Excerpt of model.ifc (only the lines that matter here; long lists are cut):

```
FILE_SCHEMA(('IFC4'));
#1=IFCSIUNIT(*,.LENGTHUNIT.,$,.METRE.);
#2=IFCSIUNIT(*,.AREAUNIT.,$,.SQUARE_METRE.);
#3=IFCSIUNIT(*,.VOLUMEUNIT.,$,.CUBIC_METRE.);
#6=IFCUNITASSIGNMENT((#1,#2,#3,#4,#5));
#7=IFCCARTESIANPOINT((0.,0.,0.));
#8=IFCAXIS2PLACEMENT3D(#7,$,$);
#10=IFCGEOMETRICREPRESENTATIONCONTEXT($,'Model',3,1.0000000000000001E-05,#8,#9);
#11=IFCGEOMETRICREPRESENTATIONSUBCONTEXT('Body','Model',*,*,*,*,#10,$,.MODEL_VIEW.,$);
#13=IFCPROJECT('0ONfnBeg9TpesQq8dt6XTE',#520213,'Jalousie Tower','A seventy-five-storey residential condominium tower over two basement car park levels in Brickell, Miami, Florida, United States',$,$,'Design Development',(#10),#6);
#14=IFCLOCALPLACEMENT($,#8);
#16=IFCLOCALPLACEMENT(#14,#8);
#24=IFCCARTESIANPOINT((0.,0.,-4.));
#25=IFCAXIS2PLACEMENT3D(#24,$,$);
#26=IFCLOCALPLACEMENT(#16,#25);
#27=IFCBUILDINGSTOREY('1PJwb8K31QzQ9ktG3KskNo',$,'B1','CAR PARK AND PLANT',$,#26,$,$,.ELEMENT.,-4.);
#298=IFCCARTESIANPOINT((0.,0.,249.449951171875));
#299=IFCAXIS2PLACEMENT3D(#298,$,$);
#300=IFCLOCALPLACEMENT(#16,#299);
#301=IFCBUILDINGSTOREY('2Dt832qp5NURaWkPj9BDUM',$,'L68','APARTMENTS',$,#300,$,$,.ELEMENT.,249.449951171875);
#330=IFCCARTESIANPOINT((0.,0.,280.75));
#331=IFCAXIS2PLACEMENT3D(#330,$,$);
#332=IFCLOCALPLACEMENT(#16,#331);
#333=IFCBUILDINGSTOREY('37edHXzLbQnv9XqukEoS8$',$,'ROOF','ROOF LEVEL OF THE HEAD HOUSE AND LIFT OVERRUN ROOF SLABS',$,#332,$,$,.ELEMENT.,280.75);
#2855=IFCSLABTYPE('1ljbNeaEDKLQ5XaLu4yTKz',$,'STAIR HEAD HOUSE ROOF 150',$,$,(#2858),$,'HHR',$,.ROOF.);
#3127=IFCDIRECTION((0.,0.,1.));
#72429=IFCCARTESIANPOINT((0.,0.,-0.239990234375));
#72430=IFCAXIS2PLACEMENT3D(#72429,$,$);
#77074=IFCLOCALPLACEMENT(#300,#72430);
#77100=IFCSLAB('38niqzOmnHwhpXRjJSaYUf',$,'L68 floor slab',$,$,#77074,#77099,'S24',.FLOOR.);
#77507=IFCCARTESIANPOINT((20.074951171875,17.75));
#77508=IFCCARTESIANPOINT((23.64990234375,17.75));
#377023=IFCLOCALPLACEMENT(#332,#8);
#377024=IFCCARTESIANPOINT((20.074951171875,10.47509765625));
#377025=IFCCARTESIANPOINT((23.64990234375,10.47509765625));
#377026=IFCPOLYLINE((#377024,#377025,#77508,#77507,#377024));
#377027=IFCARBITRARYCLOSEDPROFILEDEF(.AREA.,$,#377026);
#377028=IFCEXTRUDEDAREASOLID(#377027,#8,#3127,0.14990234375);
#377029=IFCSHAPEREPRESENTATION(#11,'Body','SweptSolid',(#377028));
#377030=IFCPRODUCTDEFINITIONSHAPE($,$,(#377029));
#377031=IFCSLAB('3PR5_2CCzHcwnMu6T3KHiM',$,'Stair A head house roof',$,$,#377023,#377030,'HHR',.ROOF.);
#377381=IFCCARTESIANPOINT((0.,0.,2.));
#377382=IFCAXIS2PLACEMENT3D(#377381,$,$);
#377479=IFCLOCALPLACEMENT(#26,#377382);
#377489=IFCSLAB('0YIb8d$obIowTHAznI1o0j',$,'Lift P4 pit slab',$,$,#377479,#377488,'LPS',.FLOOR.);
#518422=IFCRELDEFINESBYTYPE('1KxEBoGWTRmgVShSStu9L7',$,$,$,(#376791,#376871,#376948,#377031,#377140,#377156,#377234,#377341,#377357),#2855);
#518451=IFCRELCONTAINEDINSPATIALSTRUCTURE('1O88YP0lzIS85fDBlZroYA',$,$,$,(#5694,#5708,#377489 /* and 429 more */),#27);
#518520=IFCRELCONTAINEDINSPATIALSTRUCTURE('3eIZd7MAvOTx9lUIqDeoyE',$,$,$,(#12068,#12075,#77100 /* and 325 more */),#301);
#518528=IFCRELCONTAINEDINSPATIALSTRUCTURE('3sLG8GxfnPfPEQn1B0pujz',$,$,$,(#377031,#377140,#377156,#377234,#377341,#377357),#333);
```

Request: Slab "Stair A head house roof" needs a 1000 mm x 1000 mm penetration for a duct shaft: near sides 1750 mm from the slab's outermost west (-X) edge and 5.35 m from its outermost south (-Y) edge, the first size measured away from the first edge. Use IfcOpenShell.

```python
import numpy as np
import ifcopenshell
import ifcopenshell.api.feature
import ifcopenshell.api.geometry
import ifcopenshell.api.root
import ifcopenshell.geom
import ifcopenshell.util.placement
import ifcopenshell.util.representation
import ifcopenshell.util.shape
import ifcopenshell.util.unit

model = ifcopenshell.open("model.ifc")
unit_scale = ifcopenshell.util.unit.calculate_unit_scale(model)
settings = ifcopenshell.geom.settings()


def volume(element):
    """Net volume in cubic metres, openings subtracted."""
    shape = ifcopenshell.geom.create_shape(settings, element)
    return ifcopenshell.util.shape.get_volume(shape.geometry)


slab = model.by_guid("3PR5_2CCzHcwnMu6T3KHiM")
before = volume(slab)

# Extent in the slab's own axes, in metres. The edges named are its -X and -Y sides.
slab_shape = ifcopenshell.geom.create_shape(settings, slab)
vertices = ifcopenshell.util.shape.get_vertices(slab_shape.geometry)
x_min, y_min, bottom = vertices.min(axis=0)
top = vertices[:, 2].max()

opening = ifcopenshell.api.root.create_entity(model, ifc_class="IfcOpeningElement", name="Duct shaft opening", predefined_type="OPENING")
context = ifcopenshell.util.representation.get_context(model, "Model", "Body", "MODEL_VIEW")
width, depth = 1, 1
outline = [(0.0, 0.0), (width, 0.0), (width, depth), (0.0, depth), (0.0, 0.0)]
# Overshoot both faces by 50 mm so the cut is clean.
shape = ifcopenshell.api.geometry.add_slab_representation(
    model, context=context, depth=top - bottom + 0.1, polyline=outline
)
ifcopenshell.api.geometry.assign_representation(model, product=opening, representation=shape)

matrix = ifcopenshell.util.placement.get_local_placement(slab.ObjectPlacement)
matrix[:, 3] = matrix @ np.append(np.array([x_min + 1.75, y_min + 5.35, bottom - 0.05]) / unit_scale, 1.0)
ifcopenshell.api.geometry.edit_object_placement(model, product=opening, matrix=matrix, is_si=False)
ifcopenshell.api.feature.add_feature(model, feature=opening, element=slab)

after = volume(slab)

print(f"slab volume {before:.3f} -> {after:.3f} m3")

model.write("model-out.ifc")
```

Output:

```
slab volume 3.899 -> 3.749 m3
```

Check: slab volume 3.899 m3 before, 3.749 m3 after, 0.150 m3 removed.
